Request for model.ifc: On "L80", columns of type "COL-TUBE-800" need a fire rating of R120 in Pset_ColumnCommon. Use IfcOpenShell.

First a look at what the model holds.

```python
import ifcopenshell
import ifcopenshell.util.element

model = ifcopenshell.open("model.ifc")
print(model.schema)
storey = next(s for s in model.by_type("IfcBuildingStorey") if s.Name == "L80")
columns = [e for e in ifcopenshell.util.element.get_decomposition(storey) if e.is_a("IfcColumn")]
seen = {}
for e in columns:
    element_type = ifcopenshell.util.element.get_type(e)
    key = (element_type.Name if element_type != e and element_type else None, ifcopenshell.util.element.get_pset(e, "Pset_ColumnCommon", "FireRating"))
    seen[key] = seen.get(key, 0) + 1
for (name, value), count in sorted(seen.items(), key=str):
    print(count, "x", name, "|", value)
```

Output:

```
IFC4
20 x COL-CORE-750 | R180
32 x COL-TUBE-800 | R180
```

```python
import ifcopenshell
import ifcopenshell.api.pset
import ifcopenshell.util.element

model = ifcopenshell.open("model.ifc")

storey = next(s for s in model.by_type("IfcBuildingStorey") if s.Name == "L80")
columns = [e for e in ifcopenshell.util.element.get_decomposition(storey) if e.is_a("IfcColumn")]

count = 0
for e in columns:
    element_type = ifcopenshell.util.element.get_type(e)
    if element_type in (None, e) or element_type.Name != "COL-TUBE-800":
        continue
    found = ifcopenshell.util.element.get_pset(e, "Pset_ColumnCommon", should_inherit=False)
    if found:
        pset = model.by_id(found["id"])
        if len(ifcopenshell.util.element.get_elements_by_pset(pset)) > 1:
            pset = ifcopenshell.api.pset.unshare_pset(model, products=[e], pset=pset)[0]
    else:
        pset = ifcopenshell.api.pset.add_pset(model, product=e, name="Pset_ColumnCommon")
    ifcopenshell.api.pset.edit_pset(model, pset=pset, properties={"FireRating": "R120"})
    count += 1

print(count, "columns updated")

model.write("model_updated.ifc")
```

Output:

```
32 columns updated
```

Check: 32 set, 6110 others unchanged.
